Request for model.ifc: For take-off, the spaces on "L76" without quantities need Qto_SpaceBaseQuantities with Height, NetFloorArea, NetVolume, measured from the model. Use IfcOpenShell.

First a look at what the model holds.

```python
import ifcopenshell
import ifcopenshell.util.element
import ifcopenshell.util.unit

model = ifcopenshell.open("model.ifc")
print(model.schema)
for unit_type in ("LENGTHUNIT", "AREAUNIT", "VOLUMEUNIT"):
    print(unit_type, ifcopenshell.util.unit.calculate_unit_scale(model, unit_type))
storey = next(s for s in model.by_type("IfcBuildingStorey") if s.Name == "L76")
spaces = [e for e in ifcopenshell.util.element.get_decomposition(storey) if e.is_a("IfcSpace")]
for e in sorted(spaces, key=lambda e: e.id()):
    print(e.id(), e.is_a(), e.Name, list(ifcopenshell.util.element.get_psets(e, qtos_only=True)), sep=" | ")
```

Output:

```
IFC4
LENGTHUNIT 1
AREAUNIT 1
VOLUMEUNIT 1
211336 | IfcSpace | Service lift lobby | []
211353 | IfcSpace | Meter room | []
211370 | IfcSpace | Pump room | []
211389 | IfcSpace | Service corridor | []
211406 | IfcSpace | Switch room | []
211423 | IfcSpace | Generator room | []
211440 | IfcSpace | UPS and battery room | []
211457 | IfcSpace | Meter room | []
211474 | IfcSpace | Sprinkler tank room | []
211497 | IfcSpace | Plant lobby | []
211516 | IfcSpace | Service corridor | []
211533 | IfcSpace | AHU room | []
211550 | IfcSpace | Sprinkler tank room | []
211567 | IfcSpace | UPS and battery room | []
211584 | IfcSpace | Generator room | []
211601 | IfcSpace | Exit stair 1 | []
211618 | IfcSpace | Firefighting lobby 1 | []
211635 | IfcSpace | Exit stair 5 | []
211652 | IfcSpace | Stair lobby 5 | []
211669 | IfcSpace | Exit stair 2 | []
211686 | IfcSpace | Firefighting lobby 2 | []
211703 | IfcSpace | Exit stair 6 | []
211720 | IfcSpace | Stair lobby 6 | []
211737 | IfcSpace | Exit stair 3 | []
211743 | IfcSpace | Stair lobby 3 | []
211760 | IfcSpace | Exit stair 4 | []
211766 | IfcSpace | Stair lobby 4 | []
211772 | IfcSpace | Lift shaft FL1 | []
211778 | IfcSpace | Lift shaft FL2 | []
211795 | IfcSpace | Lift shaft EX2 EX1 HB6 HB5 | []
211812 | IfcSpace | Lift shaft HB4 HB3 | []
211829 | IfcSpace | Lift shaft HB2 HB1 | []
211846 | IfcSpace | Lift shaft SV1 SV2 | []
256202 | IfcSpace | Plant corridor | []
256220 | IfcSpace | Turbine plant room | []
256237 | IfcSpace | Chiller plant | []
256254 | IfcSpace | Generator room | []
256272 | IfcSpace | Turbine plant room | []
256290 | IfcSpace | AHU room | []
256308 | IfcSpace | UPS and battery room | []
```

```python
import ifcopenshell
import ifcopenshell.api.pset
import ifcopenshell.geom
import ifcopenshell.util.element
import ifcopenshell.util.shape
import ifcopenshell.util.unit

model = ifcopenshell.open("model.ifc")
unit_scale = ifcopenshell.util.unit.calculate_unit_scale(model)
area_scale = ifcopenshell.util.unit.calculate_unit_scale(model, "AREAUNIT")
volume_scale = ifcopenshell.util.unit.calculate_unit_scale(model, "VOLUMEUNIT")
settings = ifcopenshell.geom.settings()

storey = next(s for s in model.by_type("IfcBuildingStorey") if s.Name == "L76")
spaces = [e for e in ifcopenshell.util.element.get_decomposition(storey) if e.is_a("IfcSpace")]

for e in sorted(spaces, key=lambda e: e.id()):
    if ifcopenshell.util.element.get_psets(e, qtos_only=True, should_inherit=False):
        continue
    # Geometry comes back in metres, in the element's own axes.
    shape = ifcopenshell.geom.create_shape(settings, e)
    values = {
        "Height": ifcopenshell.util.shape.get_z(shape.geometry) / unit_scale,
        "NetFloorArea": ifcopenshell.util.shape.get_footprint_area(shape.geometry) / area_scale,
        "NetVolume": ifcopenshell.util.shape.get_volume(shape.geometry) / volume_scale,
    }
    qto = ifcopenshell.api.pset.add_qto(model, product=e, name="Qto_SpaceBaseQuantities")
    ifcopenshell.api.pset.edit_qto(model, qto=qto, properties=values)
    print(e.id(), {k: round(v, 3) for k, v in values.items()})

model.write("model_v2.ifc")
```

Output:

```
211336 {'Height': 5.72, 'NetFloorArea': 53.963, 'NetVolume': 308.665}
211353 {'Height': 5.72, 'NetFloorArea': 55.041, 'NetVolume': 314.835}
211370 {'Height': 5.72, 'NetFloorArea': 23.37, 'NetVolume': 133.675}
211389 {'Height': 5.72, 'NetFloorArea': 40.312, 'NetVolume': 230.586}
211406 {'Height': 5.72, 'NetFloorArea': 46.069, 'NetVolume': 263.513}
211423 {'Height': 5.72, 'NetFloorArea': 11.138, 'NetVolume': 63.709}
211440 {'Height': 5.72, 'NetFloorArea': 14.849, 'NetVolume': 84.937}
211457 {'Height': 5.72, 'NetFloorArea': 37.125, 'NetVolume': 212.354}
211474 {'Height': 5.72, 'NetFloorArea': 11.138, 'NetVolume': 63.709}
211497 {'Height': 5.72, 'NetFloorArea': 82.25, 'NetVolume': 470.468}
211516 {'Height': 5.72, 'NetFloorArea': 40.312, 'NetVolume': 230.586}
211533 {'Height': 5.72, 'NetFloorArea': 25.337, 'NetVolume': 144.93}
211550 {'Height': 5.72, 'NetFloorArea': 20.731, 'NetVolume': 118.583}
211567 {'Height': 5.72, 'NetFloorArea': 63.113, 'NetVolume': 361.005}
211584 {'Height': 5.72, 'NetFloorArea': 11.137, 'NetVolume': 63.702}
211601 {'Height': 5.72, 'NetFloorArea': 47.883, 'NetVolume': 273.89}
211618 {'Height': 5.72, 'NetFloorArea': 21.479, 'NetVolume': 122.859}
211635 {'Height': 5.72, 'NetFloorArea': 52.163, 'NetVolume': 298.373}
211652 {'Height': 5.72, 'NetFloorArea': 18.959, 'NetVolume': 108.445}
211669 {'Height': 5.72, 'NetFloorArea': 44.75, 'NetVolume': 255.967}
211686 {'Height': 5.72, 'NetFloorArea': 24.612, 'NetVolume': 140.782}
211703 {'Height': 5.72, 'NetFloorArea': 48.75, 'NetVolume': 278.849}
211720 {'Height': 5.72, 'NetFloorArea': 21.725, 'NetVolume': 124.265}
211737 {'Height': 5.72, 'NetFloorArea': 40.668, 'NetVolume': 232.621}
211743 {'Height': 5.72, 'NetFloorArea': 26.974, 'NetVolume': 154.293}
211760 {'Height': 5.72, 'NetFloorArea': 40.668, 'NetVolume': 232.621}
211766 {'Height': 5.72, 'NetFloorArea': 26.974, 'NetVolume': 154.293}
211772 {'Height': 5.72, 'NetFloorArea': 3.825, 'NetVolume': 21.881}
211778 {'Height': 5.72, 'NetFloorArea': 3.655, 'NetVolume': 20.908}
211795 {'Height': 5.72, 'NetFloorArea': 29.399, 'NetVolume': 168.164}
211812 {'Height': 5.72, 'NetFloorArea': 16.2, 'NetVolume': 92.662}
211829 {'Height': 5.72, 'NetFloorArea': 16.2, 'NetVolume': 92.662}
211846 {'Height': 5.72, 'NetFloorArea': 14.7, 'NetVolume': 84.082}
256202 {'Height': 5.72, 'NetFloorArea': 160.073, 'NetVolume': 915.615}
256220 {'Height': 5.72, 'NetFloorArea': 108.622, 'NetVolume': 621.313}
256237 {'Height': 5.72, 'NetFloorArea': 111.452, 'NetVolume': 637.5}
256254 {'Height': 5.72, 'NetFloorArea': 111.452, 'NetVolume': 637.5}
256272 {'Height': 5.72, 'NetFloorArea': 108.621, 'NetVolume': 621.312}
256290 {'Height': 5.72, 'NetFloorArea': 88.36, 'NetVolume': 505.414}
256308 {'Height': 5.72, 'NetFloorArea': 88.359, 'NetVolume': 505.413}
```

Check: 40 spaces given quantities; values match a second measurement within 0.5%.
